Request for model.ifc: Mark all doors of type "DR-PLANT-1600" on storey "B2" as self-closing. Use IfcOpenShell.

First a look at what the model holds.

```python
import ifcopenshell
import ifcopenshell.util.element

model = ifcopenshell.open("model.ifc")
print(model.schema)
storey = next(s for s in model.by_type("IfcBuildingStorey") if s.Name == "B2")
doors = [e for e in ifcopenshell.util.element.get_decomposition(storey) if e.is_a("IfcDoor")]
seen = {}
for e in doors:
    element_type = ifcopenshell.util.element.get_type(e)
    key = (element_type.Name if element_type != e and element_type else None, ifcopenshell.util.element.get_pset(e, "Pset_DoorCommon", "SelfClosing"))
    seen[key] = seen.get(key, 0) + 1
for (name, value), count in sorted(seen.items(), key=str):
    print(count, "x", name, "|", value)
```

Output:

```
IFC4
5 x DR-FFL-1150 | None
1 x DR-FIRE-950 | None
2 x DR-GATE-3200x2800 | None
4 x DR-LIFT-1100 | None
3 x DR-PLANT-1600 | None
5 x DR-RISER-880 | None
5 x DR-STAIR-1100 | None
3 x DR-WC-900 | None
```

```python
import ifcopenshell
import ifcopenshell.api.pset
import ifcopenshell.util.element

model = ifcopenshell.open("model.ifc")

storey = next(s for s in model.by_type("IfcBuildingStorey") if s.Name == "B2")
doors = [e for e in ifcopenshell.util.element.get_decomposition(storey) if e.is_a("IfcDoor")]

count = 0
for e in doors:
    element_type = ifcopenshell.util.element.get_type(e)
    if element_type in (None, e) or element_type.Name != "DR-PLANT-1600":
        continue
    # add_pset returns the element's existing set when there is one.
    pset = ifcopenshell.api.pset.add_pset(model, product=e, name="Pset_DoorCommon")
    ifcopenshell.api.pset.edit_pset(model, pset=pset, properties={"SelfClosing": True})
    count += 1

print(count, "doors updated")

model.write("model-out.ifc")
```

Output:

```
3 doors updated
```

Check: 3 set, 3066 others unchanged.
